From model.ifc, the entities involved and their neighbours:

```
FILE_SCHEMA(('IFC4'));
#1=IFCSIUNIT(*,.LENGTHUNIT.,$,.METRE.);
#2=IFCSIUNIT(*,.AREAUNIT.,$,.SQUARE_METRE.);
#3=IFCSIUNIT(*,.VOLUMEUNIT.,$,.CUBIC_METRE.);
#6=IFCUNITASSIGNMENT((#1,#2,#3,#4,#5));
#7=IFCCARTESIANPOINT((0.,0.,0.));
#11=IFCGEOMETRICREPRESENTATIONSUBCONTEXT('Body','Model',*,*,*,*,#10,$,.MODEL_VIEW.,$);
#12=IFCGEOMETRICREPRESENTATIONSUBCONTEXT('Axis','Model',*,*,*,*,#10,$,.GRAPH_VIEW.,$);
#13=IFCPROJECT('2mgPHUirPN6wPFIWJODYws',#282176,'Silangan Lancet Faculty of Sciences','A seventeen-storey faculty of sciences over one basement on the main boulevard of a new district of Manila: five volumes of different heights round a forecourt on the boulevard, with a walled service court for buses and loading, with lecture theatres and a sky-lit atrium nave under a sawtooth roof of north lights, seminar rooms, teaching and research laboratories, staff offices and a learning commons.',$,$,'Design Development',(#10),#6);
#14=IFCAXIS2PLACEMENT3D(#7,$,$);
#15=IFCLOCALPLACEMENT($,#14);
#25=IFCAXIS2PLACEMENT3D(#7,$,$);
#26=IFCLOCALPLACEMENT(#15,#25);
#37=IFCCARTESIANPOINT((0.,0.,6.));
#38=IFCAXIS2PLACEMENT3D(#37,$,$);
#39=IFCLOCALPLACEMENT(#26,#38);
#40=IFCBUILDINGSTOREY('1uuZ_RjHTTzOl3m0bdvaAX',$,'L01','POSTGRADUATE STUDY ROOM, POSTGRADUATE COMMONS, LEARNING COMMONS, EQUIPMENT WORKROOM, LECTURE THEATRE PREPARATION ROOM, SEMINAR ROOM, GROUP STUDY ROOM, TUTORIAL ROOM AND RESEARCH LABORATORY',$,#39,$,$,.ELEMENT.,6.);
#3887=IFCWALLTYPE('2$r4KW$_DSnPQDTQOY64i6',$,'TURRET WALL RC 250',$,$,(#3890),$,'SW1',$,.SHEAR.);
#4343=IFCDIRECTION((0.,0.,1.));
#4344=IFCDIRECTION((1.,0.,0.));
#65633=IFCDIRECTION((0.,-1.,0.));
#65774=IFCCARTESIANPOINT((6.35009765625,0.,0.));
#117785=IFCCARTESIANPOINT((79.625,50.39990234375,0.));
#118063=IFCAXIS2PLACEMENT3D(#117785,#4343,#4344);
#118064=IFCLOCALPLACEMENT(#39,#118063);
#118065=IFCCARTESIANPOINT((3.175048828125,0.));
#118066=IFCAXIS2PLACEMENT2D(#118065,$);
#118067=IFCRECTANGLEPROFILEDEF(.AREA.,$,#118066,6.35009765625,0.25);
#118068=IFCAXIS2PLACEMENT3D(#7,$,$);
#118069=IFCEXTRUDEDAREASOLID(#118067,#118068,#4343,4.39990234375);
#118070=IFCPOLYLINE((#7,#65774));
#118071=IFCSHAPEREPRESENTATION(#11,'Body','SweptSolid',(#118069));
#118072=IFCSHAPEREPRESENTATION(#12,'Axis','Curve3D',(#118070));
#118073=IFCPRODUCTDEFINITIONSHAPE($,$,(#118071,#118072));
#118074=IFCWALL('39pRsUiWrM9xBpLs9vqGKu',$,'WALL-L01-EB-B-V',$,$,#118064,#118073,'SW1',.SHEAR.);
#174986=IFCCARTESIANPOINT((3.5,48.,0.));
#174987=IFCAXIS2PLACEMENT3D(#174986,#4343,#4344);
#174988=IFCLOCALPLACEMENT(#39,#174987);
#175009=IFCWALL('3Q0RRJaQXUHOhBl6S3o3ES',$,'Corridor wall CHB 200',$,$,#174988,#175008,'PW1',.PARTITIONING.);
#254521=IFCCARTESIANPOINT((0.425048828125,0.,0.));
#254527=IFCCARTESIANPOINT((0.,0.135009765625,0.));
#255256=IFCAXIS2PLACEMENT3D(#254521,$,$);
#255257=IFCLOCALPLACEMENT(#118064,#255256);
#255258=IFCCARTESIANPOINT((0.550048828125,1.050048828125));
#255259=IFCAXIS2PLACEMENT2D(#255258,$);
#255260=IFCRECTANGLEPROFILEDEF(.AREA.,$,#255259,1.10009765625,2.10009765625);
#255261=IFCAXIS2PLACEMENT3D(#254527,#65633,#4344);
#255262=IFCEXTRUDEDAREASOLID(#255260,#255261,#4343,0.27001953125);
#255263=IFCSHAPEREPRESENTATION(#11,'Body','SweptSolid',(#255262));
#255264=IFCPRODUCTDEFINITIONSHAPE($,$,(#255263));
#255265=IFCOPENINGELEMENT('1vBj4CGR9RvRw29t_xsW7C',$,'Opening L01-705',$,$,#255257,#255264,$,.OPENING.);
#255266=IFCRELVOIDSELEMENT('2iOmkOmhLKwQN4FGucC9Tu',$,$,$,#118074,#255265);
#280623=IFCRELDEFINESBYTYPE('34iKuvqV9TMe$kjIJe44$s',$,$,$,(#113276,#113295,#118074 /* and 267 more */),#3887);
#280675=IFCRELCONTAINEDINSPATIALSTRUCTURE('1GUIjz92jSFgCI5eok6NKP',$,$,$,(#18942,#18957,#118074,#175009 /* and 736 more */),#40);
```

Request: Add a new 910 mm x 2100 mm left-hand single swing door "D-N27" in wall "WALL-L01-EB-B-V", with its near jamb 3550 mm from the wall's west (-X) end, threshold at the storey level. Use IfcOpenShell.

```python
import numpy as np
import ifcopenshell
import ifcopenshell.api.feature
import ifcopenshell.api.geometry
import ifcopenshell.api.root
import ifcopenshell.api.spatial
import ifcopenshell.geom
import ifcopenshell.util.element
import ifcopenshell.util.placement
import ifcopenshell.util.representation
import ifcopenshell.util.shape
import ifcopenshell.util.unit

model = ifcopenshell.open("model.ifc")
unit_scale = ifcopenshell.util.unit.calculate_unit_scale(model)
settings = ifcopenshell.geom.settings()


def volume(element):
    """Net volume in cubic metres, openings subtracted."""
    shape = ifcopenshell.geom.create_shape(settings, element)
    return ifcopenshell.util.shape.get_volume(shape.geometry)


wall = model.by_id(118074)
storey = ifcopenshell.util.element.get_container(wall, ifc_class="IfcBuildingStorey")
context = ifcopenshell.util.representation.get_context(model, "Model", "Body", "MODEL_VIEW")
before = volume(wall)

width, height, from_end, sill = 0.91, 2.1, 3.55, 0.0  # metres

# The wall runs along its own X axis, and the end named is its -X end.
wall_shape = ifcopenshell.geom.create_shape(settings, wall)
x, y, z = ifcopenshell.util.shape.get_vertices(wall_shape.geometry).T
start = x.min() + from_end
face, thickness = float(y.min()), float(y.max() - y.min())
wall_matrix = ifcopenshell.util.placement.get_local_placement(wall.ObjectPlacement)
level = ifcopenshell.util.placement.get_local_placement(storey.ObjectPlacement)[2, 3]


def in_wall(x, y):
    """Placement at x, y metres in the wall's axes, at sill height."""
    matrix = wall_matrix.copy()
    matrix[:, 3] = wall_matrix @ np.array([x / unit_scale, y / unit_scale, 0.0, 1.0])
    matrix[2, 3] = level + sill / unit_scale
    return matrix


# Opening: a box that overshoots both wall faces by 50 mm.
opening = ifcopenshell.api.root.create_entity(model, ifc_class="IfcOpeningElement", predefined_type="OPENING")
box = ifcopenshell.api.geometry.add_wall_representation(
    model, context=context, length=width, height=height, thickness=thickness + 0.1
)
ifcopenshell.api.geometry.assign_representation(model, product=opening, representation=box)
ifcopenshell.api.geometry.edit_object_placement(model, product=opening, matrix=in_wall(start, face - 0.05), is_si=False)
ifcopenshell.api.feature.add_feature(model, feature=opening, element=wall)

door = ifcopenshell.api.root.create_entity(model, ifc_class="IfcDoor", name="D-N27", predefined_type="DOOR")
door.OverallWidth, door.OverallHeight = width / unit_scale, height / unit_scale
door.OperationType = "SINGLE_SWING_LEFT"
body = ifcopenshell.api.geometry.add_door_representation(
    model,
    context=context,
    overall_width=door.OverallWidth,
    overall_height=door.OverallHeight,
    operation_type="SINGLE_SWING_LEFT",
    lining_properties={"LiningDepth": thickness / unit_scale, "ThresholdDepth": thickness / unit_scale},
)
ifcopenshell.api.geometry.assign_representation(model, product=door, representation=body)
ifcopenshell.api.spatial.assign_container(model, products=[door], relating_structure=storey)
ifcopenshell.api.feature.add_filling(model, opening=opening, element=door)

# The lining spans the wall, so the door starts at the wall face.
ifcopenshell.api.geometry.edit_object_placement(model, product=door, matrix=in_wall(start, face), is_si=False)

after = volume(wall)

print(f"wall volume {before:.3f} -> {after:.3f} m3")

model.write("model_edited.ifc")
```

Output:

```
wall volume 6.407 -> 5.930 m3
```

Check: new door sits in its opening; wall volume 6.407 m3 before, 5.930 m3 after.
